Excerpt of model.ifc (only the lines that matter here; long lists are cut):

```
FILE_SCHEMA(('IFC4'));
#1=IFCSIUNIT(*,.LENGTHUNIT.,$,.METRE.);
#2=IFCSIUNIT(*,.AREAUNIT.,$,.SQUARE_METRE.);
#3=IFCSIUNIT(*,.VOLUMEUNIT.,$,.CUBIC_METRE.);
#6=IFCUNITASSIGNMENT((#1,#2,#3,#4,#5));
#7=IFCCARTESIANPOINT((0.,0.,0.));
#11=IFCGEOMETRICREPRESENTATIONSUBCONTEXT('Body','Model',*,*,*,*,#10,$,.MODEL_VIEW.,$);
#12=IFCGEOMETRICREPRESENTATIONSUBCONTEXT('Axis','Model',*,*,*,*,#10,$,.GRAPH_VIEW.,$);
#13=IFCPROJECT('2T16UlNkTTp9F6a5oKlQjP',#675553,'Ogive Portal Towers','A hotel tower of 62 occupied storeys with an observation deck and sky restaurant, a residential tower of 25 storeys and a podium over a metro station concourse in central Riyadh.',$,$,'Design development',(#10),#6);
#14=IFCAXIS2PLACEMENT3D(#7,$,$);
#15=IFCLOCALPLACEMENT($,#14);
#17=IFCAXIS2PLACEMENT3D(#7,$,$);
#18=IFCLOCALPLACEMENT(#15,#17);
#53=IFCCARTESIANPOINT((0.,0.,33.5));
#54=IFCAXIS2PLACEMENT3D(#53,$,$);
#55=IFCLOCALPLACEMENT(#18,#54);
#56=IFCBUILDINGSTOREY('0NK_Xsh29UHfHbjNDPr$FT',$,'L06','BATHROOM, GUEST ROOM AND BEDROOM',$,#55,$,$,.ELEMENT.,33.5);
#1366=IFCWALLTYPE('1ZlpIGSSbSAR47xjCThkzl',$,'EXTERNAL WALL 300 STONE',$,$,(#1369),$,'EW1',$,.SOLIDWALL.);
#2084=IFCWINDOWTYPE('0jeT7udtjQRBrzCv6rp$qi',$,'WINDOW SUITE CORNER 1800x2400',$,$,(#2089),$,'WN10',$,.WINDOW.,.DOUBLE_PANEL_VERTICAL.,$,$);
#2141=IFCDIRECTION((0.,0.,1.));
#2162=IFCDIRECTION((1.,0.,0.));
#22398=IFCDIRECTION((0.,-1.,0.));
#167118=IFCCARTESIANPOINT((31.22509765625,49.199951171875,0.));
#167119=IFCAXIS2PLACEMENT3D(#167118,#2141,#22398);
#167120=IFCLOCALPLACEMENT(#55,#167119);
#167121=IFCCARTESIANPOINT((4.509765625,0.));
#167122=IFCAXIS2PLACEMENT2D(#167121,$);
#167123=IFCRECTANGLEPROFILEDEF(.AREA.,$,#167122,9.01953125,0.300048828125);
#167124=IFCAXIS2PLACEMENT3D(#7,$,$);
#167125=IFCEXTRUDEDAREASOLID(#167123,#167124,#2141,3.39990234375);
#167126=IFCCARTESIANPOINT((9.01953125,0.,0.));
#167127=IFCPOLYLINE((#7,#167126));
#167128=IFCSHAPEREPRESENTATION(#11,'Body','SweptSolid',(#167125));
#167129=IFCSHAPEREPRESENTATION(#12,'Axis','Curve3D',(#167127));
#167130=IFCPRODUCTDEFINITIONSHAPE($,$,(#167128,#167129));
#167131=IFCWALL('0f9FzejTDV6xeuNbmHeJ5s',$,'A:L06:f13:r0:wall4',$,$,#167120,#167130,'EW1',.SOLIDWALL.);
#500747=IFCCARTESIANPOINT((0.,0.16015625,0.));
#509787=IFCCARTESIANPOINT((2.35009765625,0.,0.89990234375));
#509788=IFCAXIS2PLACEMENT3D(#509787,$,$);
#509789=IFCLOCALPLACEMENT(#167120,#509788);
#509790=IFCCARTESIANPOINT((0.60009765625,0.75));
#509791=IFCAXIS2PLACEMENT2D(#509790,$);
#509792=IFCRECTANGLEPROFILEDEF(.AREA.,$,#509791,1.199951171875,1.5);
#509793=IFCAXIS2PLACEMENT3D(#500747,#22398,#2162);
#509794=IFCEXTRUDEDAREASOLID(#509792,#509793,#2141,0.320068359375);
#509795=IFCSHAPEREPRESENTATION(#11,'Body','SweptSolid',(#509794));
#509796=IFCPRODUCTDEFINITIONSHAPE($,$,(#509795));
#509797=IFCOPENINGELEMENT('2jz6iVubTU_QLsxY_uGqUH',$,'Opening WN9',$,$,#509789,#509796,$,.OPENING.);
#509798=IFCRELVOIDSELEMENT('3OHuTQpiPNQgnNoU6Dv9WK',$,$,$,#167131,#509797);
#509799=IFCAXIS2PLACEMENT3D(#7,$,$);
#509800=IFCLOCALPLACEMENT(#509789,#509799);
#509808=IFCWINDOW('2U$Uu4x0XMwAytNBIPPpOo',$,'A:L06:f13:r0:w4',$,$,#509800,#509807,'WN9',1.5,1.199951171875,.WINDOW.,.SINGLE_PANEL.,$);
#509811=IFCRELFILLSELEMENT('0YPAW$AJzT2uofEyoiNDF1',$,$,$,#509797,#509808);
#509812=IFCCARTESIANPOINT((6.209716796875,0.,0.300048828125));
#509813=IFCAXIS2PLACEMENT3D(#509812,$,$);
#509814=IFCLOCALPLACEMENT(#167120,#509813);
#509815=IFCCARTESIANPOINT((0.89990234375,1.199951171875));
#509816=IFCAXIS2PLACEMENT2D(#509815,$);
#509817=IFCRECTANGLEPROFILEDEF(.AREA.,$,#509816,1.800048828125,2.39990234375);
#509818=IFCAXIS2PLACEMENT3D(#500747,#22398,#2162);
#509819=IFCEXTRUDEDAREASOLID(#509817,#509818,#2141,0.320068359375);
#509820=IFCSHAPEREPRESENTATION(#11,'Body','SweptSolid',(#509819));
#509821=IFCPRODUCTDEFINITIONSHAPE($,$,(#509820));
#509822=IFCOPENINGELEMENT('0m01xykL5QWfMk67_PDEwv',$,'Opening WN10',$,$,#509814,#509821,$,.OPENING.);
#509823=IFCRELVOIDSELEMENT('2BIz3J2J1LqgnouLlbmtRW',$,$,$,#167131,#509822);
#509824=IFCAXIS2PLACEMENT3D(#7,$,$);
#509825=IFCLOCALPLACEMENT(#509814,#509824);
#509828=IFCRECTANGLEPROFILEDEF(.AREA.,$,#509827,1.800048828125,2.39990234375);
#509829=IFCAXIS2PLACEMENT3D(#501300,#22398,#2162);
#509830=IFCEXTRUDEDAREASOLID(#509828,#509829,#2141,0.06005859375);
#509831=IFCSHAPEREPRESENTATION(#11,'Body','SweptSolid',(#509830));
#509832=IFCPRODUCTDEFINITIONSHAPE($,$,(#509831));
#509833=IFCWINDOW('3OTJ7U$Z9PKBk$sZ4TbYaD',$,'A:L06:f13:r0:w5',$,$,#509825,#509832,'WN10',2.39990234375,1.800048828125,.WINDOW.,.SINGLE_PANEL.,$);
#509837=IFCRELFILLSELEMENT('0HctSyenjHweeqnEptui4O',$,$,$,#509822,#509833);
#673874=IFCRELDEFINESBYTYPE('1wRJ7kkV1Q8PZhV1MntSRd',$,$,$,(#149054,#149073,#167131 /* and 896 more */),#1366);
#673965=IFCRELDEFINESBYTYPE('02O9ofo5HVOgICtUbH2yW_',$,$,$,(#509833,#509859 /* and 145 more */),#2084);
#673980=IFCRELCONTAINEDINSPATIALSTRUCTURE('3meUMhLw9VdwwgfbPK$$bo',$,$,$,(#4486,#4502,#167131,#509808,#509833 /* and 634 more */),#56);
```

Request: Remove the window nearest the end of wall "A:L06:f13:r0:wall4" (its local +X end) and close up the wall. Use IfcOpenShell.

```python
import ifcopenshell
import ifcopenshell.api.feature
import ifcopenshell.api.root
import ifcopenshell.geom
import ifcopenshell.util.shape

model = ifcopenshell.open("model.ifc")
settings = ifcopenshell.geom.settings()


def volume(element):
    """Net volume in cubic metres, openings subtracted."""
    shape = ifcopenshell.geom.create_shape(settings, element)
    return ifcopenshell.util.shape.get_volume(shape.geometry)


window = model.by_guid("3OTJ7U$Z9PKBk$sZ4TbYaD")
opening = window.FillsVoids[0].RelatingOpeningElement
wall = opening.VoidsElements[0].RelatingBuildingElement
before = volume(wall)

ifcopenshell.api.root.remove_product(model, product=window)
ifcopenshell.api.feature.remove_feature(model, feature=opening)

after = volume(wall)

print(f"wall volume {before:.3f} -> {after:.3f} m3")

model.write("model-out.ifc")
```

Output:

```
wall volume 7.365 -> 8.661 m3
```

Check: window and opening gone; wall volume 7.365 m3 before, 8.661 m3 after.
